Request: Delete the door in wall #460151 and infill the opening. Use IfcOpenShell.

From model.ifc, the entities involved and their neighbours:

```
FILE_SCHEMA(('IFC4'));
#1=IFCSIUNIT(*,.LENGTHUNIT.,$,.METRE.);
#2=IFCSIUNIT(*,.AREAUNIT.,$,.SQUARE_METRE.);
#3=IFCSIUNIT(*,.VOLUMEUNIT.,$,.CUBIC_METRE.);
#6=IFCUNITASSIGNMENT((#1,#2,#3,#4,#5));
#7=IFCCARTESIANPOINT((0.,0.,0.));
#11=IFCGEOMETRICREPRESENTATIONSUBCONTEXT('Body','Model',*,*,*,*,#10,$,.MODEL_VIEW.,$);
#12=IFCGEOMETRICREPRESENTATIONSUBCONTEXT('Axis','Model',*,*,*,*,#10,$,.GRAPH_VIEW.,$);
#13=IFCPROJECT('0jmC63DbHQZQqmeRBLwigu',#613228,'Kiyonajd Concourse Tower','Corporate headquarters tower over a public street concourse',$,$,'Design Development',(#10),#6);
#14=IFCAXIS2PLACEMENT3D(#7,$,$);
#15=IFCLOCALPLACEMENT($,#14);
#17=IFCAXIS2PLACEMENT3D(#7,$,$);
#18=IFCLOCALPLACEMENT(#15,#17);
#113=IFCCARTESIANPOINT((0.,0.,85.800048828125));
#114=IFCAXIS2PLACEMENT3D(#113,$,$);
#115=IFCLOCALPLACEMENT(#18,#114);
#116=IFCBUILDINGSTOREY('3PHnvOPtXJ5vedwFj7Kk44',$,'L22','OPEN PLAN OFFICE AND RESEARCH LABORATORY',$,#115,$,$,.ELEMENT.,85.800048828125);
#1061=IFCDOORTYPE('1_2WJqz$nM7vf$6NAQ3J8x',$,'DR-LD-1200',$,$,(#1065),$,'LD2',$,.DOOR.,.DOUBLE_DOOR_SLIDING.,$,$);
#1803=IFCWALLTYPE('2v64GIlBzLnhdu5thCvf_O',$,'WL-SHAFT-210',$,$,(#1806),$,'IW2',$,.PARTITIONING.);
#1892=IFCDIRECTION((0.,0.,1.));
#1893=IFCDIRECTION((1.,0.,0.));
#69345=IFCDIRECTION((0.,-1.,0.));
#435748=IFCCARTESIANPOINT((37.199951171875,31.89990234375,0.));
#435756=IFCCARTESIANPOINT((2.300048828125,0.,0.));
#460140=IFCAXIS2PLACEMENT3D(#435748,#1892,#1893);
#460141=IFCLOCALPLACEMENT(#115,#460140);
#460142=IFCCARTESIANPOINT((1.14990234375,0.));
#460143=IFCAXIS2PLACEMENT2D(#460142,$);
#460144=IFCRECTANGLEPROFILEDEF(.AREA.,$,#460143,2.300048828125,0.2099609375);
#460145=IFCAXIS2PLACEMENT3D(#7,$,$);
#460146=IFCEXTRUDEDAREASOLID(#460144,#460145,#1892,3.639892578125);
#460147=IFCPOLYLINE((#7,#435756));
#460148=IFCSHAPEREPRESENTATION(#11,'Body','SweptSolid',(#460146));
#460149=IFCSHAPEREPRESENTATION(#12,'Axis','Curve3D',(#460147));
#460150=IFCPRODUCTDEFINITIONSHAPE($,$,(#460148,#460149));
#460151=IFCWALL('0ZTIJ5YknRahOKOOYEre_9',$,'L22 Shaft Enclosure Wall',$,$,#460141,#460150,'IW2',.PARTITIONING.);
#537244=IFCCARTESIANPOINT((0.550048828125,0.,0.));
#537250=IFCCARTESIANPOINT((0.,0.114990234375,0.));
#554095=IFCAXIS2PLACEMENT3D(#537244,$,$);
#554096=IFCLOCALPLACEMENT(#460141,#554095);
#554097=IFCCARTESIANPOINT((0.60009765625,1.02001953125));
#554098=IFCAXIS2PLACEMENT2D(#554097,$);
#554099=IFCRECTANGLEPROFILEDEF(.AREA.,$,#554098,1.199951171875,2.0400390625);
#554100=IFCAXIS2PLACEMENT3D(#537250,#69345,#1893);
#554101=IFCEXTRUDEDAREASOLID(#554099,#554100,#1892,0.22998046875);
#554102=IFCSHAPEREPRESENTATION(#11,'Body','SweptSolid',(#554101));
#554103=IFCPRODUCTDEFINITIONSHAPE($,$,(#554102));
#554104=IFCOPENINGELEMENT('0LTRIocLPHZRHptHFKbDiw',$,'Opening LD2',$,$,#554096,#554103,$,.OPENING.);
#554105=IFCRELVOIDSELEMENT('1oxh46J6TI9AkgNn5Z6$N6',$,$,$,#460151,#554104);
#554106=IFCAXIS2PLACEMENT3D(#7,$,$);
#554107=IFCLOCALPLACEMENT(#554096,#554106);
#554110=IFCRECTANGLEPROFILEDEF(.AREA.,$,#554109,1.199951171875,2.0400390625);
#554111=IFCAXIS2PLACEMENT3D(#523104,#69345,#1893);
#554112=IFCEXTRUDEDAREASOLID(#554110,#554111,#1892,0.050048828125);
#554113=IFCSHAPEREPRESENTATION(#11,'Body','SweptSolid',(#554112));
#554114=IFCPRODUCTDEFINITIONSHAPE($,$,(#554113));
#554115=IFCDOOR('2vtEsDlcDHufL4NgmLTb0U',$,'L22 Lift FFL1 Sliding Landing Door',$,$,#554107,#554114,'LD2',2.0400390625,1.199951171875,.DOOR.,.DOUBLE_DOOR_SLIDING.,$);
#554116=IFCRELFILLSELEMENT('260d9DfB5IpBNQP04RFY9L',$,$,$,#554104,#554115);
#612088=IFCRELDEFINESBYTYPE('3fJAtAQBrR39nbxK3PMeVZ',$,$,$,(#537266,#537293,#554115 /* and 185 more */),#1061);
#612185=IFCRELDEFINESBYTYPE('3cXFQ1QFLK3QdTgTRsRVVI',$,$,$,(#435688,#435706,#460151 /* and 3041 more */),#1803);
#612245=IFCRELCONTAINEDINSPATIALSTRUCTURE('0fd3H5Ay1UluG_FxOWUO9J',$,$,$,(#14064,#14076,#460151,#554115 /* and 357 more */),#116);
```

```python
import ifcopenshell
import ifcopenshell.api.feature
import ifcopenshell.api.root
import ifcopenshell.geom
import ifcopenshell.util.shape

model = ifcopenshell.open("model.ifc")
settings = ifcopenshell.geom.settings()


def volume(element):
    """Net volume in cubic metres, openings subtracted."""
    shape = ifcopenshell.geom.create_shape(settings, element)
    return ifcopenshell.util.shape.get_volume(shape.geometry)


door = model.by_guid("2vtEsDlcDHufL4NgmLTb0U")
opening = door.FillsVoids[0].RelatingOpeningElement
wall = opening.VoidsElements[0].RelatingBuildingElement
before = volume(wall)

ifcopenshell.api.root.remove_product(model, product=door)
ifcopenshell.api.feature.remove_feature(model, feature=opening)

after = volume(wall)

print(f"wall volume {before:.3f} -> {after:.3f} m3")

model.write("model_edited.ifc")
```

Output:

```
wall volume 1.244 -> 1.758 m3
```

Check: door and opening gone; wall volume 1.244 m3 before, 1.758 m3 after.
